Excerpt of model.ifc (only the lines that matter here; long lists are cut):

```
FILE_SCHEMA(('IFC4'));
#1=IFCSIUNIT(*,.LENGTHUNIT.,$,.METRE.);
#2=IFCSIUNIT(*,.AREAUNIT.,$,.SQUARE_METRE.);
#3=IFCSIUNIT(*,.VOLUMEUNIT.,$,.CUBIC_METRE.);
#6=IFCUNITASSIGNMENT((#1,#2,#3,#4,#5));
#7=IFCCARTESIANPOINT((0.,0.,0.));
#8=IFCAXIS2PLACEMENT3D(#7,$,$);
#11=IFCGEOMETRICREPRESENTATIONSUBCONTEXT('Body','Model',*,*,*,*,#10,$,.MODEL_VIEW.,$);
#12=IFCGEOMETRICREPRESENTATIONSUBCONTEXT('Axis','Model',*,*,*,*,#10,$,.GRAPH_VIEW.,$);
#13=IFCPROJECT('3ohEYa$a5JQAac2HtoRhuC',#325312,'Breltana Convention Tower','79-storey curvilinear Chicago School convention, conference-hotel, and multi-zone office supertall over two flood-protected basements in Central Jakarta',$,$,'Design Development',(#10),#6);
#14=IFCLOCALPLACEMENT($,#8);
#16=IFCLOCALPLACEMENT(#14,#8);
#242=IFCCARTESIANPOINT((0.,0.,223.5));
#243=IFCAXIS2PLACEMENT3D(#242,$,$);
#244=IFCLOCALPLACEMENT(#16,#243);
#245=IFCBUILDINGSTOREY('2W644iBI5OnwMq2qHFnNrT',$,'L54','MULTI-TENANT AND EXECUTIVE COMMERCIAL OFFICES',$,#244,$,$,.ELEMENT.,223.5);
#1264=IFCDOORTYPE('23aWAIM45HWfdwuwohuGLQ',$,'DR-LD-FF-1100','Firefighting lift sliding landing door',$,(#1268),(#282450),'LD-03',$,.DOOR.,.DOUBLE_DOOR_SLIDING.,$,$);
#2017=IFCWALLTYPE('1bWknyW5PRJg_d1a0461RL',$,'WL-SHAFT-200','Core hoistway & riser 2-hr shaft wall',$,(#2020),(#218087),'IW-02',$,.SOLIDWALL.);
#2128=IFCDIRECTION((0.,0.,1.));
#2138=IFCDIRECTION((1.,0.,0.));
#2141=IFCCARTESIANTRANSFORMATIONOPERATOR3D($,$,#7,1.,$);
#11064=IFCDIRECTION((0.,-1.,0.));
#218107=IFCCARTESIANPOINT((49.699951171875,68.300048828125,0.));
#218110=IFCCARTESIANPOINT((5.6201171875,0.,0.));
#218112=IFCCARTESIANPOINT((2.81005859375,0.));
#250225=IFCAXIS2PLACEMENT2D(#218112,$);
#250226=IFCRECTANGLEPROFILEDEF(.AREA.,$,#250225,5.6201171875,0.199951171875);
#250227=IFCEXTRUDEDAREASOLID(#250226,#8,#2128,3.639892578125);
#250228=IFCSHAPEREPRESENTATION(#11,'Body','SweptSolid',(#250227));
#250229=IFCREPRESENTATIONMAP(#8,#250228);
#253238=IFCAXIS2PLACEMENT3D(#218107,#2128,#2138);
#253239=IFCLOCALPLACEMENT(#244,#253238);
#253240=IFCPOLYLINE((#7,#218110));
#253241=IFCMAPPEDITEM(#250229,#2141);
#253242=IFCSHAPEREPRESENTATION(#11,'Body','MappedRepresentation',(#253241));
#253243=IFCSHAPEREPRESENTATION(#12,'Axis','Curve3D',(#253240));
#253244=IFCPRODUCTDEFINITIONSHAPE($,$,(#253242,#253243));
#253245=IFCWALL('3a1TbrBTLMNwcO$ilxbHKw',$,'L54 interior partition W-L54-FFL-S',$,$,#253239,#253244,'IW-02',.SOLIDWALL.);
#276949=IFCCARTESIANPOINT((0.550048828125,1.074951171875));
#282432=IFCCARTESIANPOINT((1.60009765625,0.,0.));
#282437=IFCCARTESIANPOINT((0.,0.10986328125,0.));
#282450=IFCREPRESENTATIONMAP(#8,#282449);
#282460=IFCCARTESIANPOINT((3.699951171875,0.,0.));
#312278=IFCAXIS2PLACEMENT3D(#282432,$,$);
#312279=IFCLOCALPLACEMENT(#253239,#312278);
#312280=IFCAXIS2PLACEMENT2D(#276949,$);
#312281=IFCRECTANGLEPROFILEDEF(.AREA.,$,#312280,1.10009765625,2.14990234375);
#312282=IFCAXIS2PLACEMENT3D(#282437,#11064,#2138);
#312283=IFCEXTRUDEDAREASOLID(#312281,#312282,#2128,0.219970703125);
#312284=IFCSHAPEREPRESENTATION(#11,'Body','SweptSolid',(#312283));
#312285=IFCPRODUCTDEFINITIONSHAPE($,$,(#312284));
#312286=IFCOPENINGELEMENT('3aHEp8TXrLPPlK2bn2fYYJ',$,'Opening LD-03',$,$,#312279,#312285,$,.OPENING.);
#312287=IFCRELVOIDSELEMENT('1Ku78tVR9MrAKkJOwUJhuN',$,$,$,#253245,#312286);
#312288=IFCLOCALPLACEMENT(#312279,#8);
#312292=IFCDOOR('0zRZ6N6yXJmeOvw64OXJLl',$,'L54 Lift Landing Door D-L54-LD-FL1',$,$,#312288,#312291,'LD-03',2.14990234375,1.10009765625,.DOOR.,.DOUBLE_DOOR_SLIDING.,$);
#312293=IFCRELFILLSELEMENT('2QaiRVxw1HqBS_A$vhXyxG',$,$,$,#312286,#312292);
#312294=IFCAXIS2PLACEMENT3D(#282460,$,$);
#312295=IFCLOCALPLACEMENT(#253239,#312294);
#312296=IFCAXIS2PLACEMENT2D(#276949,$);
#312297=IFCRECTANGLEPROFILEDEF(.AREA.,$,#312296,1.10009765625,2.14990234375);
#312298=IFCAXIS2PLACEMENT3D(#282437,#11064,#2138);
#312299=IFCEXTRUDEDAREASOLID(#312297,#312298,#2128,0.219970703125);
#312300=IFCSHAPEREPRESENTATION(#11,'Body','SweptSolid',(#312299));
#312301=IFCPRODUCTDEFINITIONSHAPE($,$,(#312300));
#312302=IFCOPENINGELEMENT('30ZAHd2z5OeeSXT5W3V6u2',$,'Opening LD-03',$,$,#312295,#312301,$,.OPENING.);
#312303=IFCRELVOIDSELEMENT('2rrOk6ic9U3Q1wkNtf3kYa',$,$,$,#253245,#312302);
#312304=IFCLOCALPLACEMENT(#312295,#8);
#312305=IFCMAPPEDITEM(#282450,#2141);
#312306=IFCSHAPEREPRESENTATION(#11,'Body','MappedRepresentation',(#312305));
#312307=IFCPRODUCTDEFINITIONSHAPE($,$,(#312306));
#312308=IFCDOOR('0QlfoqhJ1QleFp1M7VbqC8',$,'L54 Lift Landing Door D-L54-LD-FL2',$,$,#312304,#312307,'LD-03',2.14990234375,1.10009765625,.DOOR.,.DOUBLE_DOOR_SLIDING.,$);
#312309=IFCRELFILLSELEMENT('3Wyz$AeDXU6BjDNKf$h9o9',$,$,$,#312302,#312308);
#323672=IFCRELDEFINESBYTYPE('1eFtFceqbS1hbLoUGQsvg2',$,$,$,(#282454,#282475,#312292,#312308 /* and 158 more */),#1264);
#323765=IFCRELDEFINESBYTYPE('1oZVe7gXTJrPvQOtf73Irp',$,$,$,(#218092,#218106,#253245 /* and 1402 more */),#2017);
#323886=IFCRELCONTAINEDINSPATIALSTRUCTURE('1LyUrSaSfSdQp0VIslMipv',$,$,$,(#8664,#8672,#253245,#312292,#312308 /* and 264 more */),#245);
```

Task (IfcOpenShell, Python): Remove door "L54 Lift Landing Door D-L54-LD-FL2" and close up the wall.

```python
import ifcopenshell
import ifcopenshell.api.feature
import ifcopenshell.api.root
import ifcopenshell.geom
import ifcopenshell.util.shape

model = ifcopenshell.open("model.ifc")
settings = ifcopenshell.geom.settings()


def volume(element):
    """Net volume in cubic metres, openings subtracted."""
    shape = ifcopenshell.geom.create_shape(settings, element)
    return ifcopenshell.util.shape.get_volume(shape.geometry)


door = model.by_guid("0QlfoqhJ1QleFp1M7VbqC8")
opening = door.FillsVoids[0].RelatingOpeningElement
wall = opening.VoidsElements[0].RelatingBuildingElement
before = volume(wall)

ifcopenshell.api.root.remove_product(model, product=door)
ifcopenshell.api.feature.remove_feature(model, feature=opening)

after = volume(wall)

print(f"wall volume {before:.3f} -> {after:.3f} m3")

model.write("model_edited.ifc")
```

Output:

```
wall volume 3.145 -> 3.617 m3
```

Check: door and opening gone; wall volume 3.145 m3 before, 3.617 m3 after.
